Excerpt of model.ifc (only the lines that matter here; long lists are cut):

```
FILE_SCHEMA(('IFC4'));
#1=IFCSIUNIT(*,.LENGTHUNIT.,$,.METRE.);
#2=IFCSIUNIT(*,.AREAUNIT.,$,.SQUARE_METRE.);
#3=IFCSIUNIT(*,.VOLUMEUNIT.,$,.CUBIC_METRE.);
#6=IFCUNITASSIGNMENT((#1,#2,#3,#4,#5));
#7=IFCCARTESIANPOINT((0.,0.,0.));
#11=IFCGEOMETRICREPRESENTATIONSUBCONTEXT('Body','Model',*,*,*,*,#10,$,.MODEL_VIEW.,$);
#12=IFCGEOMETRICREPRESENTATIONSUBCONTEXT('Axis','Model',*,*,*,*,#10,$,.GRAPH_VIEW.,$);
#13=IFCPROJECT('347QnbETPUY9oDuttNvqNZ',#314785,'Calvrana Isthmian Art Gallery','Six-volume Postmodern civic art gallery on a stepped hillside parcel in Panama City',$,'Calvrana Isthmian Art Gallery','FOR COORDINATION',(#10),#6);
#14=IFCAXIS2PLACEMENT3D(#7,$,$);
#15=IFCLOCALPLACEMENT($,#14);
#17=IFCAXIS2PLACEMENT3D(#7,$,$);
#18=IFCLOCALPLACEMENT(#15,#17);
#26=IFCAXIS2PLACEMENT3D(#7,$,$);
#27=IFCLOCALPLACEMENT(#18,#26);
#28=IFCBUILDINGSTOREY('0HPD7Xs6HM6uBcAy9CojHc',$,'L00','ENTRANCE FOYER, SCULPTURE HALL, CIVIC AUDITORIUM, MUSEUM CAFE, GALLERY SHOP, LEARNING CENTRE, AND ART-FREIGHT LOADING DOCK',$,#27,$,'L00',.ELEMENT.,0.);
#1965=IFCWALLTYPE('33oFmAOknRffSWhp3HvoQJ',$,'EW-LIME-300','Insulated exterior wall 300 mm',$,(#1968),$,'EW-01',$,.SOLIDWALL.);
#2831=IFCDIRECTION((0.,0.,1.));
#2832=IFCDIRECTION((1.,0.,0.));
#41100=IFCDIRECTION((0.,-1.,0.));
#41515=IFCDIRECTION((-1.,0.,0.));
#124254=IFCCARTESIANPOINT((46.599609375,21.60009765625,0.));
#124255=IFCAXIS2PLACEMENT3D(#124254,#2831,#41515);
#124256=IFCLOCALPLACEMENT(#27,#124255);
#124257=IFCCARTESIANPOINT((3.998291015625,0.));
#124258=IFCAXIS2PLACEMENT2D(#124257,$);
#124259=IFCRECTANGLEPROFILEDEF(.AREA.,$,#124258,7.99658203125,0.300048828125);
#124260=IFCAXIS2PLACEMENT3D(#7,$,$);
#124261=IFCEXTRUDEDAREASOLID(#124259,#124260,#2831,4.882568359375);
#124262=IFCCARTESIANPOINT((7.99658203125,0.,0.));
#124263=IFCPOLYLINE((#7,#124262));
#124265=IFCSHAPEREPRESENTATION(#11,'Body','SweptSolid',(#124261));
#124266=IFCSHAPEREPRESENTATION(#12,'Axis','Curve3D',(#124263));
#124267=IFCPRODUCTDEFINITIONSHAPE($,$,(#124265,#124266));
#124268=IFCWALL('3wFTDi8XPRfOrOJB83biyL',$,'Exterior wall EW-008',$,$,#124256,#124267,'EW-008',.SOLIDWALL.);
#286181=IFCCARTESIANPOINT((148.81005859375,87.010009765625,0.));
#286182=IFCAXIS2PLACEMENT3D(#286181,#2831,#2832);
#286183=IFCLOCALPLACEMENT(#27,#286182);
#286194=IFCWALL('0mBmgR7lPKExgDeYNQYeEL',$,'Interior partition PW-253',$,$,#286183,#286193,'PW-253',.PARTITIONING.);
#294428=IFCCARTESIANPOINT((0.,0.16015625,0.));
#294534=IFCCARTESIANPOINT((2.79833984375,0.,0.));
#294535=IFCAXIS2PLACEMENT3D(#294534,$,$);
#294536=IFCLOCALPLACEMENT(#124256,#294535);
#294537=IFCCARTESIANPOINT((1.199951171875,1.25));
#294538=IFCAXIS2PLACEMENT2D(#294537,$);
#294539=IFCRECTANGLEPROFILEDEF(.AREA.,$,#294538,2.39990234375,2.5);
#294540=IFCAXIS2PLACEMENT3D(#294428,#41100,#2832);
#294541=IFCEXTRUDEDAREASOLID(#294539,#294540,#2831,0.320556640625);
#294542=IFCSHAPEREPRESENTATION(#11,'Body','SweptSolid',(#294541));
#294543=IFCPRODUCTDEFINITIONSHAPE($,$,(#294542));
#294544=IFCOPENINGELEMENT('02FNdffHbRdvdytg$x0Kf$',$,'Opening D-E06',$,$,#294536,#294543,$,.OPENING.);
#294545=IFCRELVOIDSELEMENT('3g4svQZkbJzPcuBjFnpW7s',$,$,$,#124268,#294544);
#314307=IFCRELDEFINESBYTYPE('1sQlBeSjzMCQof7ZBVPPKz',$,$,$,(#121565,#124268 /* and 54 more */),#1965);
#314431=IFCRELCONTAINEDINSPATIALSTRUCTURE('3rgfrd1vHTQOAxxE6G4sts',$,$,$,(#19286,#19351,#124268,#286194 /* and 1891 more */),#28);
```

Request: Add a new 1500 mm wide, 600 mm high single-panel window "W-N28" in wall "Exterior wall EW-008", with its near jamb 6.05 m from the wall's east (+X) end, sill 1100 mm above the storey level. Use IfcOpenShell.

```python
import numpy as np
import ifcopenshell
import ifcopenshell.api.feature
import ifcopenshell.api.geometry
import ifcopenshell.api.root
import ifcopenshell.api.spatial
import ifcopenshell.geom
import ifcopenshell.util.element
import ifcopenshell.util.placement
import ifcopenshell.util.representation
import ifcopenshell.util.shape
import ifcopenshell.util.unit

model = ifcopenshell.open("model.ifc")
unit_scale = ifcopenshell.util.unit.calculate_unit_scale(model)
settings = ifcopenshell.geom.settings()


def volume(element):
    """Net volume in cubic metres, openings subtracted."""
    shape = ifcopenshell.geom.create_shape(settings, element)
    return ifcopenshell.util.shape.get_volume(shape.geometry)


wall = model.by_guid("3wFTDi8XPRfOrOJB83biyL")
storey = ifcopenshell.util.element.get_container(wall, ifc_class="IfcBuildingStorey")
context = ifcopenshell.util.representation.get_context(model, "Model", "Body", "MODEL_VIEW")
before = volume(wall)

width, height, from_end, sill = 1.5, 0.6, 6.05, 1.1  # metres

# The wall runs along its own X axis, and the end named is its -X end.
wall_shape = ifcopenshell.geom.create_shape(settings, wall)
x, y, z = ifcopenshell.util.shape.get_vertices(wall_shape.geometry).T
start = x.min() + from_end
face, thickness = float(y.min()), float(y.max() - y.min())
wall_matrix = ifcopenshell.util.placement.get_local_placement(wall.ObjectPlacement)
level = ifcopenshell.util.placement.get_local_placement(storey.ObjectPlacement)[2, 3]


def in_wall(x, y):
    """Placement at x, y metres in the wall's axes, at sill height."""
    matrix = wall_matrix.copy()
    matrix[:, 3] = wall_matrix @ np.array([x / unit_scale, y / unit_scale, 0.0, 1.0])
    matrix[2, 3] = level + sill / unit_scale
    return matrix


# Opening: a box that overshoots both wall faces by 50 mm.
opening = ifcopenshell.api.root.create_entity(model, ifc_class="IfcOpeningElement", predefined_type="OPENING")
box = ifcopenshell.api.geometry.add_wall_representation(
    model, context=context, length=width, height=height, thickness=thickness + 0.1
)
ifcopenshell.api.geometry.assign_representation(model, product=opening, representation=box)
ifcopenshell.api.geometry.edit_object_placement(model, product=opening, matrix=in_wall(start, face - 0.05), is_si=False)
ifcopenshell.api.feature.add_feature(model, feature=opening, element=wall)

window = ifcopenshell.api.root.create_entity(model, ifc_class="IfcWindow", name="W-N28", predefined_type="WINDOW")
window.OverallWidth, window.OverallHeight = width / unit_scale, height / unit_scale
window.PartitioningType = "SINGLE_PANEL"
body = ifcopenshell.api.geometry.add_window_representation(
    model,
    context=context,
    overall_width=window.OverallWidth,
    overall_height=window.OverallHeight,
    partition_type="SINGLE_PANEL",
)
ifcopenshell.api.geometry.assign_representation(model, product=window, representation=body)
ifcopenshell.api.spatial.assign_container(model, products=[window], relating_structure=storey)
ifcopenshell.api.feature.add_filling(model, opening=opening, element=window)

# Centre the window in the wall's thickness.
ifcopenshell.api.geometry.edit_object_placement(model, product=window, matrix=in_wall(start, face), is_si=False)
window_shape = ifcopenshell.geom.create_shape(settings, window)
depth = ifcopenshell.util.shape.get_vertices(window_shape.geometry)[:, 1]
offset = face + thickness / 2 - (depth.min() + depth.max()) / 2
ifcopenshell.api.geometry.edit_object_placement(model, product=window, matrix=in_wall(start, offset), is_si=False)

after = volume(wall)

print(f"wall volume {before:.3f} -> {after:.3f} m3")

model.write("model-out.ifc")
```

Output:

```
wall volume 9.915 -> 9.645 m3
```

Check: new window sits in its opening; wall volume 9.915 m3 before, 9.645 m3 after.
